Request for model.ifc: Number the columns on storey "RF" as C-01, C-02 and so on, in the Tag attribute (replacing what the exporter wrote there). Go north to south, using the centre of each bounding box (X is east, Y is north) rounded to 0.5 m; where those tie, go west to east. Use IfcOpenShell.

First a look at what the model holds.

```python
import ifcopenshell
import ifcopenshell.util.element
import ifcopenshell.util.placement

model = ifcopenshell.open("model.ifc")
print(model.schema)
storey = next(s for s in model.by_type("IfcBuildingStorey") if s.Name == "RF")
columns = [e for e in ifcopenshell.util.element.get_decomposition(storey) if e.is_a("IfcColumn")]
for e in sorted(columns, key=lambda e: e.id()):
    origin = ifcopenshell.util.placement.get_local_placement(e.ObjectPlacement)[:3, 3]
    print(e.id(), e.Tag, e.Name, origin.round(2) + 0.0, sep=" | ")
```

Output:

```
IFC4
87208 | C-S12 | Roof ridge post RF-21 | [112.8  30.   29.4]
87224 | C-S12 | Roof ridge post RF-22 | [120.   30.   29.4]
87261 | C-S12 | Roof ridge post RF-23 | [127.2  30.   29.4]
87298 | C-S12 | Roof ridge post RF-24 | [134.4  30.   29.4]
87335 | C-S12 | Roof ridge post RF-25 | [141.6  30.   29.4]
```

```python
import ifcopenshell
import ifcopenshell.geom
import ifcopenshell.util.element
import ifcopenshell.util.shape

model = ifcopenshell.open("model.ifc")
settings = ifcopenshell.geom.settings()
settings.set("use-world-coords", True)


def centre(element):
    shape = ifcopenshell.geom.create_shape(settings, element)
    return ifcopenshell.util.shape.get_bbox_centroid(shape.geometry)


storey = next(s for s in model.by_type("IfcBuildingStorey") if s.Name == "RF")
columns = [e for e in ifcopenshell.util.element.get_decomposition(storey) if e.is_a("IfcColumn")]

# Insertion points can sit at a corner or the storey origin, so sort by the geometry (in metres).
centres = {e: centre(e) for e in columns}
columns.sort(key=lambda e: (-round(centres[e][1] / 0.5), centres[e][0]))

for i, e in enumerate(columns, start=1):
    number = f"C-{i:02d}"
    e.Tag = number
    print(e.id(), number)

model.write("model_edited.ifc")
```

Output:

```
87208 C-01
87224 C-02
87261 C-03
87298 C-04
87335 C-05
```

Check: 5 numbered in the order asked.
